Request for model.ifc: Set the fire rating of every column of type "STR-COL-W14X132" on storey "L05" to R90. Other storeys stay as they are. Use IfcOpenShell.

First a look at what the model holds.

```python
import ifcopenshell
import ifcopenshell.util.element

model = ifcopenshell.open("model.ifc")
print(model.schema)
storey = next(s for s in model.by_type("IfcBuildingStorey") if s.Name == "L05")
columns = [e for e in ifcopenshell.util.element.get_decomposition(storey) if e.is_a("IfcColumn")]
seen = {}
for e in columns:
    element_type = ifcopenshell.util.element.get_type(e)
    key = (element_type.Name if element_type != e and element_type else None, ifcopenshell.util.element.get_pset(e, "Pset_ColumnCommon", "FireRating"))
    seen[key] = seen.get(key, 0) + 1
for (name, value), count in sorted(seen.items(), key=str):
    print(count, "x", name, "|", value)
```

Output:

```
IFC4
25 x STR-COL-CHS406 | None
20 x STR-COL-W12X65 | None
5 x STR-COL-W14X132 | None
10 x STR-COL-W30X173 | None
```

```python
import ifcopenshell
import ifcopenshell.api.pset
import ifcopenshell.util.element

model = ifcopenshell.open("model.ifc")

storey = next(s for s in model.by_type("IfcBuildingStorey") if s.Name == "L05")
columns = [e for e in ifcopenshell.util.element.get_decomposition(storey) if e.is_a("IfcColumn")]

count = 0
for e in columns:
    element_type = ifcopenshell.util.element.get_type(e)
    if element_type in (None, e) or element_type.Name != "STR-COL-W14X132":
        continue
    # add_pset returns the element's existing set when there is one.
    pset = ifcopenshell.api.pset.add_pset(model, product=e, name="Pset_ColumnCommon")
    ifcopenshell.api.pset.edit_pset(model, pset=pset, properties={"FireRating": "R90"})
    count += 1

print(count, "columns updated")

model.write("model_edited.ifc")
```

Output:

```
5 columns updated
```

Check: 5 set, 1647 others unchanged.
